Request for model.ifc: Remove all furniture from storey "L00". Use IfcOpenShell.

First a look at what the model holds.

```python
import ifcopenshell
import ifcopenshell.util.element

model = ifcopenshell.open("model.ifc")
print(model.schema)
storey = next(s for s in model.by_type("IfcBuildingStorey") if s.Name == "L00")
furniture = [e for e in ifcopenshell.util.element.get_decomposition(storey) if e.is_a("IfcFurnishingElement")]
seen = {}
for e in furniture:
    element_type = ifcopenshell.util.element.get_type(e)
    name = element_type.Name if element_type not in (None, e) else None
    seen[name] = seen.get(name, 0) + 1
for name, count in sorted(seen.items(), key=str):
    print(count, "x", name)
```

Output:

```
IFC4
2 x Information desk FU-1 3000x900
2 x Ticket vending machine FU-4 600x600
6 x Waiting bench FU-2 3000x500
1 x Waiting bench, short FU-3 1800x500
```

```python
import ifcopenshell
import ifcopenshell.api.root
import ifcopenshell.util.element

model = ifcopenshell.open("model.ifc")

storey = next(s for s in model.by_type("IfcBuildingStorey") if s.Name == "L00")
furniture = [e for e in ifcopenshell.util.element.get_decomposition(storey) if e.is_a("IfcFurnishingElement")]

for e in furniture:
    ifcopenshell.api.root.remove_product(model, product=e)
print(len(furniture), "removed")

model.write("model_updated.ifc")
```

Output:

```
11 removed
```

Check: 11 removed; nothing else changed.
